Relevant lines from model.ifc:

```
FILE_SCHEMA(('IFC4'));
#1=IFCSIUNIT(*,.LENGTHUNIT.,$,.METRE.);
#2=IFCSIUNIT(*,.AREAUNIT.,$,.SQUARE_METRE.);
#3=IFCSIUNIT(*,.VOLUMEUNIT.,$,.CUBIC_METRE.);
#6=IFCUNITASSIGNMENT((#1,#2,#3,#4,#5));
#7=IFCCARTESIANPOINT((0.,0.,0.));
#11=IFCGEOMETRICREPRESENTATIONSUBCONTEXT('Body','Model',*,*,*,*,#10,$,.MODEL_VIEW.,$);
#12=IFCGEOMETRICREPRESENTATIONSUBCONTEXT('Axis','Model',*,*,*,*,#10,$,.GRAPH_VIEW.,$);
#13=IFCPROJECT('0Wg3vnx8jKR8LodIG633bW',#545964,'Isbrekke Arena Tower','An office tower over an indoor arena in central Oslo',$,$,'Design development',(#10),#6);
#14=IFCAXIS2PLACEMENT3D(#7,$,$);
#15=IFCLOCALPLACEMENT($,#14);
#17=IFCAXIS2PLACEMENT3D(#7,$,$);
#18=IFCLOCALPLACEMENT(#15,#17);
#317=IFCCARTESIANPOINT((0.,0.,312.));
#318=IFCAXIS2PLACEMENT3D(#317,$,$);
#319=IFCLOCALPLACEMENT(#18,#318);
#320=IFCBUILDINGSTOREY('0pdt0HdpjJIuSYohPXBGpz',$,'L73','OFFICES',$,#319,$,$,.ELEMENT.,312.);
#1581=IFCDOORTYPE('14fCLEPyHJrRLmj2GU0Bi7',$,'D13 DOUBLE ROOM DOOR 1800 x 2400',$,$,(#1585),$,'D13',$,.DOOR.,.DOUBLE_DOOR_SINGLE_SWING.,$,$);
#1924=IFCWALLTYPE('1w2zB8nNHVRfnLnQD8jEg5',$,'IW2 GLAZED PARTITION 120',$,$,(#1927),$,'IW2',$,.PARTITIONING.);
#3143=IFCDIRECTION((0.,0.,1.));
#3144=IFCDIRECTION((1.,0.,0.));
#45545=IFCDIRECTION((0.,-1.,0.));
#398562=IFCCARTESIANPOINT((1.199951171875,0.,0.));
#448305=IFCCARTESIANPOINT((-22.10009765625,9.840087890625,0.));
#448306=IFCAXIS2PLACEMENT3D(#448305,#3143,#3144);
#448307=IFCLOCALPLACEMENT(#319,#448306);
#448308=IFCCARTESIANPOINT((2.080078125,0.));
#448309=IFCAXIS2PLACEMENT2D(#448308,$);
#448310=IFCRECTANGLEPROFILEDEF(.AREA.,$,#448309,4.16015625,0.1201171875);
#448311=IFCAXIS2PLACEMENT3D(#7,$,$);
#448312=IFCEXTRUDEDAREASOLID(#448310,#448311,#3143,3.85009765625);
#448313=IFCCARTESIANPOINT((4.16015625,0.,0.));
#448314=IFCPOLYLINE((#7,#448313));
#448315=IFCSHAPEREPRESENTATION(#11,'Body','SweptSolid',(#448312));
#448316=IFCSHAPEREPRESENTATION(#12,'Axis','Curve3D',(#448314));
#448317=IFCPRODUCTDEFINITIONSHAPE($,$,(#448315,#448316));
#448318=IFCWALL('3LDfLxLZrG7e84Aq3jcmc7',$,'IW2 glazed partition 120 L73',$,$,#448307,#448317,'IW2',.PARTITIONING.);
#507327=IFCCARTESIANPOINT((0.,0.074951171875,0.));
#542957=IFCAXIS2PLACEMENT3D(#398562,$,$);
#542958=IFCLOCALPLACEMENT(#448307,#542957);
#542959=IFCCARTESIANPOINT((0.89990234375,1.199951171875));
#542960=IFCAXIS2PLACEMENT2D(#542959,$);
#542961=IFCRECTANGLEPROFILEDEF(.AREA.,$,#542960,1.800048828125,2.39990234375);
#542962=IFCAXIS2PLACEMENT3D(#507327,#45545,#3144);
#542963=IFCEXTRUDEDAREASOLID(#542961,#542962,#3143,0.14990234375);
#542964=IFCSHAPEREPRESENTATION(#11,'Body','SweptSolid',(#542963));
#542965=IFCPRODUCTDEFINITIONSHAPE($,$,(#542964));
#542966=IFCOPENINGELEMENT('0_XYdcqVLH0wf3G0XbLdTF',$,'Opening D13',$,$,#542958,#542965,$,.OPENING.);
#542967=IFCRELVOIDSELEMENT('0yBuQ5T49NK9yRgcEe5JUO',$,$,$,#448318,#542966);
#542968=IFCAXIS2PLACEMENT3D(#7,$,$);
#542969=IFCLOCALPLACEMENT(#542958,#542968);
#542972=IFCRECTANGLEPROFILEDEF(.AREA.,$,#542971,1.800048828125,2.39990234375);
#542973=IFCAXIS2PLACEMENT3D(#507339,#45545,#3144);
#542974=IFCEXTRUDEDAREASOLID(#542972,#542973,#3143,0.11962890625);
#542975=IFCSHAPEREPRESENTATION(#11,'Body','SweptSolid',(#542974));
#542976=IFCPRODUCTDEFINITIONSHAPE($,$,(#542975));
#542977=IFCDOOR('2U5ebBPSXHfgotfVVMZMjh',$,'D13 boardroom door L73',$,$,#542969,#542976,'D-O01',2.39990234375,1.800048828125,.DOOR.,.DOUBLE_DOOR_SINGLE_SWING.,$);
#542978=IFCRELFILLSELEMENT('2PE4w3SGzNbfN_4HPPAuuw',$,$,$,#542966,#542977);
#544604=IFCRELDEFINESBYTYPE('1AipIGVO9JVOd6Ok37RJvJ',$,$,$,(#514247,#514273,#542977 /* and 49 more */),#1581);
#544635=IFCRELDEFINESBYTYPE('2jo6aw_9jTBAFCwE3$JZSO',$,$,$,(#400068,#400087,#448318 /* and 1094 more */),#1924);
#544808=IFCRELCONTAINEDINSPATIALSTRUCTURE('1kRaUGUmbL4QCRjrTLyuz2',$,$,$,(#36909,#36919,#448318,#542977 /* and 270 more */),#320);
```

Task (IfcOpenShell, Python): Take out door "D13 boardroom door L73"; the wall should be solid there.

```python
import ifcopenshell
import ifcopenshell.api.feature
import ifcopenshell.api.root
import ifcopenshell.geom
import ifcopenshell.util.shape

model = ifcopenshell.open("model.ifc")
settings = ifcopenshell.geom.settings()


def volume(element):
    """Net volume in cubic metres, openings subtracted."""
    shape = ifcopenshell.geom.create_shape(settings, element)
    return ifcopenshell.util.shape.get_volume(shape.geometry)


door = model.by_guid("2U5ebBPSXHfgotfVVMZMjh")
opening = door.FillsVoids[0].RelatingOpeningElement
wall = opening.VoidsElements[0].RelatingBuildingElement
before = volume(wall)

ifcopenshell.api.root.remove_product(model, product=door)
ifcopenshell.api.feature.remove_feature(model, feature=opening)

after = volume(wall)

print(f"wall volume {before:.3f} -> {after:.3f} m3")

model.write("model_edited.ifc")
```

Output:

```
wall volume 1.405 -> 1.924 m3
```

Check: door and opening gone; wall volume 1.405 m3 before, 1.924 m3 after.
